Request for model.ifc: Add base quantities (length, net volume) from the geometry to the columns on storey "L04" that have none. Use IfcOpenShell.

First a look at what the model holds.

```python
import ifcopenshell
import ifcopenshell.util.element
import ifcopenshell.util.unit

model = ifcopenshell.open("model.ifc")
print(model.schema)
for unit_type in ("LENGTHUNIT", "AREAUNIT", "VOLUMEUNIT"):
    print(unit_type, ifcopenshell.util.unit.calculate_unit_scale(model, unit_type))
storey = next(s for s in model.by_type("IfcBuildingStorey") if s.Name == "L04")
columns = [e for e in ifcopenshell.util.element.get_decomposition(storey) if e.is_a("IfcColumn")]
for e in sorted(columns, key=lambda e: e.id()):
    print(e.id(), e.is_a(), e.Name, list(ifcopenshell.util.element.get_psets(e, qtos_only=True)), sep=" | ")
```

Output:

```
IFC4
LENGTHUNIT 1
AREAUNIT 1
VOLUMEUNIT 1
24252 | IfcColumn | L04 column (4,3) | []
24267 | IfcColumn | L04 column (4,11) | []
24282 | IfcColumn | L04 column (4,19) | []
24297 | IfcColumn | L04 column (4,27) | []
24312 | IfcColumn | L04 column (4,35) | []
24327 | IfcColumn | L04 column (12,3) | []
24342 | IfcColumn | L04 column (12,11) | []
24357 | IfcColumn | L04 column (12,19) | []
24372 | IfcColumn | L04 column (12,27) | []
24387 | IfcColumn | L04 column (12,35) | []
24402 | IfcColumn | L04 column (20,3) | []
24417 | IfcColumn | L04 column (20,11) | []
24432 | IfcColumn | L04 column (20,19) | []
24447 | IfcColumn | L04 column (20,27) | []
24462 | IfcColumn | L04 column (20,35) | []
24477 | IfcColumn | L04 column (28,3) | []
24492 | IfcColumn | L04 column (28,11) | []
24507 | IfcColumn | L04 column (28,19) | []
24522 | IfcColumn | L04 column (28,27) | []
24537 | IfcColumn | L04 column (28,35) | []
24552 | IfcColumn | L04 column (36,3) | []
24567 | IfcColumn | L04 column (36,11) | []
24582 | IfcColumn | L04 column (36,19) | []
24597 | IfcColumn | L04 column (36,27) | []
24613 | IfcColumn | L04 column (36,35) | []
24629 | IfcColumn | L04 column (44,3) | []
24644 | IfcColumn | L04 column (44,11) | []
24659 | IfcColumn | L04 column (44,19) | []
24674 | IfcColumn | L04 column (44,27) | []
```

```python
import ifcopenshell
import ifcopenshell.api.pset
import ifcopenshell.geom
import ifcopenshell.util.element
import ifcopenshell.util.shape
import ifcopenshell.util.unit

model = ifcopenshell.open("model.ifc")
unit_scale = ifcopenshell.util.unit.calculate_unit_scale(model)
volume_scale = ifcopenshell.util.unit.calculate_unit_scale(model, "VOLUMEUNIT")
settings = ifcopenshell.geom.settings()

storey = next(s for s in model.by_type("IfcBuildingStorey") if s.Name == "L04")
columns = [e for e in ifcopenshell.util.element.get_decomposition(storey) if e.is_a("IfcColumn")]

for e in sorted(columns, key=lambda e: e.id()):
    if ifcopenshell.util.element.get_psets(e, qtos_only=True, should_inherit=False):
        continue
    # Geometry comes back in metres, in the element's own axes.
    shape = ifcopenshell.geom.create_shape(settings, e)
    values = {
        "Length": ifcopenshell.util.shape.get_z(shape.geometry) / unit_scale,
        "NetVolume": ifcopenshell.util.shape.get_volume(shape.geometry) / volume_scale,
    }
    qto = ifcopenshell.api.pset.add_qto(model, product=e, name="Qto_ColumnBaseQuantities")
    ifcopenshell.api.pset.edit_qto(model, qto=qto, properties=values)
    print(e.id(), {k: round(v, 3) for k, v in values.items()})

model.write("model_rev.ifc")
```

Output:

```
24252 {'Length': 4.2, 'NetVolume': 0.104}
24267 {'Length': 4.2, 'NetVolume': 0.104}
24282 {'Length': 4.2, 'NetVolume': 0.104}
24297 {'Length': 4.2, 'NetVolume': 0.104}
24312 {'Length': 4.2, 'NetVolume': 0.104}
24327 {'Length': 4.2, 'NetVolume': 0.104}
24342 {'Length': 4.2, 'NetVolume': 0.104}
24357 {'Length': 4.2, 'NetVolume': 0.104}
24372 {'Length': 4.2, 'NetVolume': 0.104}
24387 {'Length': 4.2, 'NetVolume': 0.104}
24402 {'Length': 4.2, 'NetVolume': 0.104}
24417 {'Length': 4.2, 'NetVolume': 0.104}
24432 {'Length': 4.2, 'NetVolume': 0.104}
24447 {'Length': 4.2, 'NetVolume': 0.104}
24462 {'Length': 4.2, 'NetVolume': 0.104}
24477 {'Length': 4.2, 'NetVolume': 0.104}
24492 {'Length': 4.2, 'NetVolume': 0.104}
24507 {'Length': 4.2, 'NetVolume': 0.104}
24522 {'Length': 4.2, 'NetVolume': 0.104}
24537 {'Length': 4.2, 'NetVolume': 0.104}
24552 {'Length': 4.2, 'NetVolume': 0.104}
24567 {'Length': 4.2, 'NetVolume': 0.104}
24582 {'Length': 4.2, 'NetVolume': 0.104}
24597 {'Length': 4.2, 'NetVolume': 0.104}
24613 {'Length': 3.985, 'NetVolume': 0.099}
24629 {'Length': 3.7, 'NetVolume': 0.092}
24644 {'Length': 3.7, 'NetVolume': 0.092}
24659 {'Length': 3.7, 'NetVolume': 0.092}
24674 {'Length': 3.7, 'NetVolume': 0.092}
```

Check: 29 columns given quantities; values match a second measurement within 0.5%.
